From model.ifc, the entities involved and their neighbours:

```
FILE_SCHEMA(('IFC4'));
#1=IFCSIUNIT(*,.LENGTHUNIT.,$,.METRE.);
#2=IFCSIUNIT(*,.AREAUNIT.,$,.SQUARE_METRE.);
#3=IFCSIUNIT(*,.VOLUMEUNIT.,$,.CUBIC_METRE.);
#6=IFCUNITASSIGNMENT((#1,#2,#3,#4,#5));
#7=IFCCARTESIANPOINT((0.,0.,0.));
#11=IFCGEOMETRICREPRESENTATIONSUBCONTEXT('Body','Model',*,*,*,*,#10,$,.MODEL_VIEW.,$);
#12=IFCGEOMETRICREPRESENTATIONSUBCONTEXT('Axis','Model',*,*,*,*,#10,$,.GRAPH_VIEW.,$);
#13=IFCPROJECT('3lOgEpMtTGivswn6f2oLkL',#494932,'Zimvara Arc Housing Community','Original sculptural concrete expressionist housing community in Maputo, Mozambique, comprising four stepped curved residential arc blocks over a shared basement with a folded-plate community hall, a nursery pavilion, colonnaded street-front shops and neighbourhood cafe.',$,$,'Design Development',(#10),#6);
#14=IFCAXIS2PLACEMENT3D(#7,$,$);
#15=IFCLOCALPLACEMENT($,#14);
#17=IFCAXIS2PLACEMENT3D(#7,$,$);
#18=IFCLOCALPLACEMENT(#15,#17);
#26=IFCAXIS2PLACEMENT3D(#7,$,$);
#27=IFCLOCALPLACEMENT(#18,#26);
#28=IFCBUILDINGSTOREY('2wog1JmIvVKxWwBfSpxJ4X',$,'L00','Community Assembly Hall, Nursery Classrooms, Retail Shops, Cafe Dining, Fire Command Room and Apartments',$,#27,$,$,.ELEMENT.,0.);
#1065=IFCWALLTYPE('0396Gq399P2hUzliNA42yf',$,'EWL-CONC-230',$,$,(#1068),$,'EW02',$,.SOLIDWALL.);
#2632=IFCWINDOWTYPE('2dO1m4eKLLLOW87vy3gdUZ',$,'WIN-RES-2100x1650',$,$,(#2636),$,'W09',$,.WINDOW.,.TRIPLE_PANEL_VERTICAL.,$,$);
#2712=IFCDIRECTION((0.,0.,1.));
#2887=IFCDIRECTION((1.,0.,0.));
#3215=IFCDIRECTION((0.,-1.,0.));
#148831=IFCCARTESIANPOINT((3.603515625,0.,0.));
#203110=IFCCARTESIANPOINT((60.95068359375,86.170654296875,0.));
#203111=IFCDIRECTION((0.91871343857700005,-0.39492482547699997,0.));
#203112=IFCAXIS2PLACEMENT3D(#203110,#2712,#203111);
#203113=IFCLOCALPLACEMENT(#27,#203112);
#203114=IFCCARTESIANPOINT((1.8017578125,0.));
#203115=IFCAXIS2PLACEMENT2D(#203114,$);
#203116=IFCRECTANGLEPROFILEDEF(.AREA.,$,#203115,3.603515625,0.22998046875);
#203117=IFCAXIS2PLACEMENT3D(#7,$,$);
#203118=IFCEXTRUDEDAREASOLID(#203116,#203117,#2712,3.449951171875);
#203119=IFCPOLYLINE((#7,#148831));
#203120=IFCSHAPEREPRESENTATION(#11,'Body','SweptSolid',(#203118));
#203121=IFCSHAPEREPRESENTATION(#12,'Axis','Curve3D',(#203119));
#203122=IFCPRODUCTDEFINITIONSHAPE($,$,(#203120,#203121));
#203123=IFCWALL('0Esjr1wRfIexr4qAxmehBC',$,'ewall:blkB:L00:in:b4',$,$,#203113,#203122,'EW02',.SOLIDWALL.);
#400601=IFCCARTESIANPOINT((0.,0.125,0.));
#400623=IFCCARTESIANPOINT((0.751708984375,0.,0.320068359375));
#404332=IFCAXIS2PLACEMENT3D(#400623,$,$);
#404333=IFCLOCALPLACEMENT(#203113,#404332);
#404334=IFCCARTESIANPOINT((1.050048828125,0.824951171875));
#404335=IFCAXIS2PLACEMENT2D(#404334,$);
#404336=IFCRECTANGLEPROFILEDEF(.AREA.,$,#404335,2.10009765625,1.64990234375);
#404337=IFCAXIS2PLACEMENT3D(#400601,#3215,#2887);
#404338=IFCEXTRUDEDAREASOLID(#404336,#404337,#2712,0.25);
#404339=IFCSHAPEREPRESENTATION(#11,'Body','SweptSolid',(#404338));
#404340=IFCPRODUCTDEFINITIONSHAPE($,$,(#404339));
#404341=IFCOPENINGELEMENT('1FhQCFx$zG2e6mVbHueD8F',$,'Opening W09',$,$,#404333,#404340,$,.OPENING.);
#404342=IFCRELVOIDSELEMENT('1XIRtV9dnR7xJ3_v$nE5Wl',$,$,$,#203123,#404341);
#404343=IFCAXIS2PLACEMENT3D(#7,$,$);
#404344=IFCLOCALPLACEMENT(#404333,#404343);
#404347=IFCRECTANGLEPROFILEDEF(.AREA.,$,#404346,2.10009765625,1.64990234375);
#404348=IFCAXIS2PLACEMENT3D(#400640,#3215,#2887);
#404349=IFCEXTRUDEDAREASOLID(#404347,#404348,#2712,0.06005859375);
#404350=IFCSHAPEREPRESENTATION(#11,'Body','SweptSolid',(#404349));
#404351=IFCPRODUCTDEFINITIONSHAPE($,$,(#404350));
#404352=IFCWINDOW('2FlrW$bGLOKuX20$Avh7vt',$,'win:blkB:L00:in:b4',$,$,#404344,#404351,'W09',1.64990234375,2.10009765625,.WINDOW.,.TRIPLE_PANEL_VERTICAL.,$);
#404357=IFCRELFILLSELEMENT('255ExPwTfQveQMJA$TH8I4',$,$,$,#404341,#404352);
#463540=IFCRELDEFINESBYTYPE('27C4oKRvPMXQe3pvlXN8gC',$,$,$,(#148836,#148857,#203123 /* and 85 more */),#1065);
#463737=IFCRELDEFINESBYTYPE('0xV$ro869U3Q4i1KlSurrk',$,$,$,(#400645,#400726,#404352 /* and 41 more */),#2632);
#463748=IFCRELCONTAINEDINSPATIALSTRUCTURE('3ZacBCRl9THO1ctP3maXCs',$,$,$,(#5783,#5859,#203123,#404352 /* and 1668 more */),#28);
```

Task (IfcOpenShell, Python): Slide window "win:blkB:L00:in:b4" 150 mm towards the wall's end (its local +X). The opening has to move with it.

```python
import ifcopenshell
import ifcopenshell.api.geometry
import ifcopenshell.util.placement
import ifcopenshell.util.unit

model = ifcopenshell.open("model.ifc")
unit_scale = ifcopenshell.util.unit.calculate_unit_scale(model)

window = model.by_guid("2FlrW$bGLOKuX20$Avh7vt")
opening = window.FillsVoids[0].RelatingOpeningElement
wall = opening.VoidsElements[0].RelatingBuildingElement

wall_matrix = ifcopenshell.util.placement.get_local_placement(wall.ObjectPlacement)
shift = wall_matrix[:3, 0] * 0.15 / unit_scale
before = ifcopenshell.util.placement.get_local_placement(window.ObjectPlacement)[:3, 3].copy()

# The window is placed relative to its opening, so it follows when the opening moves.
matrix = ifcopenshell.util.placement.get_local_placement(opening.ObjectPlacement)
matrix[:3, 3] += shift
ifcopenshell.api.geometry.edit_object_placement(
    model, product=opening, matrix=matrix, is_si=False, should_transform_children=True
)

after = ifcopenshell.util.placement.get_local_placement(window.ObjectPlacement)[:3, 3]
print("window moved by", (after - before).round(3) + 0.0)

model.write("model_rev.ifc")
```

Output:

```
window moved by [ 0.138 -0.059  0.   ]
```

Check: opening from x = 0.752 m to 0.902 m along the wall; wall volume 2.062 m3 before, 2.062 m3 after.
